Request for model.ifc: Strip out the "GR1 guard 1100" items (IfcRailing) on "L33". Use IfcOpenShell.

First a look at what the model holds.

```python
import ifcopenshell
import ifcopenshell.util.element

model = ifcopenshell.open("model.ifc")
print(model.schema)
storey = next(s for s in model.by_type("IfcBuildingStorey") if s.Name == "L33")
railings = [e for e in ifcopenshell.util.element.get_decomposition(storey) if e.is_a("IfcRailing")]
seen = {}
for e in railings:
    element_type = ifcopenshell.util.element.get_type(e)
    name = element_type.Name if element_type not in (None, e) else None
    seen[name] = seen.get(name, 0) + 1
for name, count in sorted(seen.items(), key=str):
    print(count, "x", name)
```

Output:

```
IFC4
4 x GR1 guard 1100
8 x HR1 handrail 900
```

```python
import ifcopenshell
import ifcopenshell.api.root
import ifcopenshell.util.element

model = ifcopenshell.open("model.ifc")

storey = next(s for s in model.by_type("IfcBuildingStorey") if s.Name == "L33")
railings = [e for e in ifcopenshell.util.element.get_decomposition(storey) if e.is_a("IfcRailing")]
targets = [e for e in railings if (t := ifcopenshell.util.element.get_type(e)) not in (None, e) and t.Name == "GR1 guard 1100"]

for e in targets:
    ifcopenshell.api.root.remove_product(model, product=e)
print(len(targets), "removed")

model.write("model_rev.ifc")
```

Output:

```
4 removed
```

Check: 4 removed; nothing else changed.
